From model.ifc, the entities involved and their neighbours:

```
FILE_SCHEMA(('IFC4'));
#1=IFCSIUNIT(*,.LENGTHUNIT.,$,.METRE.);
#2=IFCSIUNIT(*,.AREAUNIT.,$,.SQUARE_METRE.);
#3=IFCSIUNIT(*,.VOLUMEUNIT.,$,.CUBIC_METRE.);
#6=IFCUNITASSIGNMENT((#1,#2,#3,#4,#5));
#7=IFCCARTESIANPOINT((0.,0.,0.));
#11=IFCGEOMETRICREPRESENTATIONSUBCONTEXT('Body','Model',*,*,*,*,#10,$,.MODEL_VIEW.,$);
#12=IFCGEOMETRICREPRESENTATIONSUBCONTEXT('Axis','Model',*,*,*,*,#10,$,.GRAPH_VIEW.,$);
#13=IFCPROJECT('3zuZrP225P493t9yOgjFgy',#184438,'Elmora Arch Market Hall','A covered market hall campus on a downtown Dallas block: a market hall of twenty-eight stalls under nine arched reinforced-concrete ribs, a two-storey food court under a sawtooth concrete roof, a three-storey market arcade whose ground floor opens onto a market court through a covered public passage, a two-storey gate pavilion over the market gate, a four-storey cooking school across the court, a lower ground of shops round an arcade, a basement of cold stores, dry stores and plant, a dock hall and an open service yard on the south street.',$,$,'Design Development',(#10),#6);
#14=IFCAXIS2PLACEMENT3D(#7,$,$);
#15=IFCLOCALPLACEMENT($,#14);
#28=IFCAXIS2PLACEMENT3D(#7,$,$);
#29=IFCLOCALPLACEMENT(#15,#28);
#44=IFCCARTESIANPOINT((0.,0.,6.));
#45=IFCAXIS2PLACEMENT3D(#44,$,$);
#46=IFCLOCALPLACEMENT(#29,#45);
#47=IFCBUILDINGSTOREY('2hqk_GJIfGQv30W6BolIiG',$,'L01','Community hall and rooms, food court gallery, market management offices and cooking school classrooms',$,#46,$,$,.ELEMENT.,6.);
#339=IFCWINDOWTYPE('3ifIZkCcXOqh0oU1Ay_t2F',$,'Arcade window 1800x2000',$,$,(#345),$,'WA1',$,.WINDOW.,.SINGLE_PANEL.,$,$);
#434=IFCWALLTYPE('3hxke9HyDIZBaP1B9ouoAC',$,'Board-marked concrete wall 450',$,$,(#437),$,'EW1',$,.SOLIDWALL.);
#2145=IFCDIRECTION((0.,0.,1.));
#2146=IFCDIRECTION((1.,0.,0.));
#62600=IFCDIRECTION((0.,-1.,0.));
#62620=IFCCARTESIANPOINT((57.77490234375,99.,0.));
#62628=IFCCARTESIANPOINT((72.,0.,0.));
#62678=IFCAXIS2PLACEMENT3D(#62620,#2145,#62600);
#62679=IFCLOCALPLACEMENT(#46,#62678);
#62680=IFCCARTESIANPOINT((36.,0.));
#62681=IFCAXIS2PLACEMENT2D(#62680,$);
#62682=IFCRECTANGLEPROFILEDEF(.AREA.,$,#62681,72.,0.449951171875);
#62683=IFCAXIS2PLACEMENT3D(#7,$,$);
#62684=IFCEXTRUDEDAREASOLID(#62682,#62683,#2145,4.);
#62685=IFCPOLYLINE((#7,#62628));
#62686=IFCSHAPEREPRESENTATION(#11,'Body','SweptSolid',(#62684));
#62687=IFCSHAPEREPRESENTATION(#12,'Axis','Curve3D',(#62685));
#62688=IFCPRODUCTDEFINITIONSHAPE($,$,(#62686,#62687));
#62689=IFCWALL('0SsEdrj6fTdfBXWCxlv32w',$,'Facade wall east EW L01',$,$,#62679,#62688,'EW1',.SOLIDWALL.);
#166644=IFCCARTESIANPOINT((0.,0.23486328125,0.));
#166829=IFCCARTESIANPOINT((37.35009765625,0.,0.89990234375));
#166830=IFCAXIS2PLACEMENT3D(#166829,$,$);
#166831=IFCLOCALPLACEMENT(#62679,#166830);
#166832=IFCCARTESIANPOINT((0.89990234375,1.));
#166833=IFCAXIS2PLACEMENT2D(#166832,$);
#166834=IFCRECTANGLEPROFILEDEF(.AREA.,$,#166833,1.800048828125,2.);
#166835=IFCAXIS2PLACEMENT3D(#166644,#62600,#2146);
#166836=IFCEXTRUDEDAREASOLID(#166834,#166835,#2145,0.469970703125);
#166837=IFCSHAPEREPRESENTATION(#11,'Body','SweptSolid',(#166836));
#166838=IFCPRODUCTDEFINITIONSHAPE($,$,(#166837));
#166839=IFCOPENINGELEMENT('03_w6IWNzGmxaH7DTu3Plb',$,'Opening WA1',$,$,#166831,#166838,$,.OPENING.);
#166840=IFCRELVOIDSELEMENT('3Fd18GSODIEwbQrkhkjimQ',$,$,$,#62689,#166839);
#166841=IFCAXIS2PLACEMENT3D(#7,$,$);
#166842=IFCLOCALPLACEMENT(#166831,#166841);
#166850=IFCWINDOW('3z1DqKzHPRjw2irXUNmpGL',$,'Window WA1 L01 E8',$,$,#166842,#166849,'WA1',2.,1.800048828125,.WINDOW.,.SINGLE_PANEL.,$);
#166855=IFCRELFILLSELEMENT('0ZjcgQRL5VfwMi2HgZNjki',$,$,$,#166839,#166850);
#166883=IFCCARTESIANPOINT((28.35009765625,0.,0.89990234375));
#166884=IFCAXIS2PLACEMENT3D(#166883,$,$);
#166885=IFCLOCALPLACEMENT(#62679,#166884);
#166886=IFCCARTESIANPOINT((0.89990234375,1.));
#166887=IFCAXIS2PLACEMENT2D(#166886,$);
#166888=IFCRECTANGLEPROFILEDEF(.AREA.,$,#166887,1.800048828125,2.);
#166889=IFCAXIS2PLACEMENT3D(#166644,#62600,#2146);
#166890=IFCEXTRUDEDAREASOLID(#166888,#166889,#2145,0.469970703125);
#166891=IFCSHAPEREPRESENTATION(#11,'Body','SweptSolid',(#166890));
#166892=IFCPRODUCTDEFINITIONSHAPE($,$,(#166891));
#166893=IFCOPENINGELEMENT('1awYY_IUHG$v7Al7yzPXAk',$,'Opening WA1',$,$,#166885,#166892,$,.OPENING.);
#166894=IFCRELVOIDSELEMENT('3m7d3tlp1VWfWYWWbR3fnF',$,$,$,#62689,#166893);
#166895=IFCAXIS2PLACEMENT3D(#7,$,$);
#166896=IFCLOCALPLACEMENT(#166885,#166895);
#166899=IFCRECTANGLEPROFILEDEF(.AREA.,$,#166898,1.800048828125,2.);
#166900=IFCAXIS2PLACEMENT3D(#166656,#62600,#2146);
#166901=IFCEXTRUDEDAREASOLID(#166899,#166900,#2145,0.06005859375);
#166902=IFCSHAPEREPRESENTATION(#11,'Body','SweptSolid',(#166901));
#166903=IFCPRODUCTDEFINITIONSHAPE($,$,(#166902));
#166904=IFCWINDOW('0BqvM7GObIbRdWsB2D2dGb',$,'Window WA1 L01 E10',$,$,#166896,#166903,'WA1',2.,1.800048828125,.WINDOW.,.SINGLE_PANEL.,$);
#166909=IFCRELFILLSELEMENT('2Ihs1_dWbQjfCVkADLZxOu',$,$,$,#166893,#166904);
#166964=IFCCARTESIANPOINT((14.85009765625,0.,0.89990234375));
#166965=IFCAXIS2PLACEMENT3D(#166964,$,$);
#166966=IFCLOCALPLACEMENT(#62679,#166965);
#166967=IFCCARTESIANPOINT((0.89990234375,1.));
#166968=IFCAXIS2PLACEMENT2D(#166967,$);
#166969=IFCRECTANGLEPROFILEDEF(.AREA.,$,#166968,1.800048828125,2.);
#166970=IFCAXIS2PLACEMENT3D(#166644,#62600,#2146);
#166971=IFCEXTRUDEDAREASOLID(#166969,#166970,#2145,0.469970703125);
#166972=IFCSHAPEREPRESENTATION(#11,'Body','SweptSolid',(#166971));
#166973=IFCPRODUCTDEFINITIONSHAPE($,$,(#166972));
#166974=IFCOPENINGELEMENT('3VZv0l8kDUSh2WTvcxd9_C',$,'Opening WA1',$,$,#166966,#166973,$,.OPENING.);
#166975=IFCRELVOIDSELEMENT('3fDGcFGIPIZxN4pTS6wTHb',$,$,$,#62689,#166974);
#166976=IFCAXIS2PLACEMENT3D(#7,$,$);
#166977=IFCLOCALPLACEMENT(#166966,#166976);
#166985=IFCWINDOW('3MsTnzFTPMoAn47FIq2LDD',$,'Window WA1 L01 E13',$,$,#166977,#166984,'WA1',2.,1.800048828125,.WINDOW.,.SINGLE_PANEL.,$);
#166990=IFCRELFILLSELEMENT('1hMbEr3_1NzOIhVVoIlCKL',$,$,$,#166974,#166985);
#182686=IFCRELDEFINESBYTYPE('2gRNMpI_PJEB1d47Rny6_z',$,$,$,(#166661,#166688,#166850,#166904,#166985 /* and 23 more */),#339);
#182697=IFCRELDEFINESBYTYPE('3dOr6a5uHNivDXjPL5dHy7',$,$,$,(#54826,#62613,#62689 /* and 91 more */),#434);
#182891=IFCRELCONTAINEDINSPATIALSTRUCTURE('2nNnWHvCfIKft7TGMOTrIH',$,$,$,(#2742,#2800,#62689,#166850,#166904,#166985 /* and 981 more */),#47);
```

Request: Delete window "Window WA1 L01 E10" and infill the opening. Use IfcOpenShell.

```python
import ifcopenshell
import ifcopenshell.api.feature
import ifcopenshell.api.root
import ifcopenshell.geom
import ifcopenshell.util.shape

model = ifcopenshell.open("model.ifc")
settings = ifcopenshell.geom.settings()


def volume(element):
    """Net volume in cubic metres, openings subtracted."""
    shape = ifcopenshell.geom.create_shape(settings, element)
    return ifcopenshell.util.shape.get_volume(shape.geometry)


window = model.by_guid("0BqvM7GObIbRdWsB2D2dGb")
opening = window.FillsVoids[0].RelatingOpeningElement
wall = opening.VoidsElements[0].RelatingBuildingElement
before = volume(wall)

ifcopenshell.api.root.remove_product(model, product=window)
ifcopenshell.api.feature.remove_feature(model, feature=opening)

after = volume(wall)

print(f"wall volume {before:.3f} -> {after:.3f} m3")

model.write("model_v2.ifc")
```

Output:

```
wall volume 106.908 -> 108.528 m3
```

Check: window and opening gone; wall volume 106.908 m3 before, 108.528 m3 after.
